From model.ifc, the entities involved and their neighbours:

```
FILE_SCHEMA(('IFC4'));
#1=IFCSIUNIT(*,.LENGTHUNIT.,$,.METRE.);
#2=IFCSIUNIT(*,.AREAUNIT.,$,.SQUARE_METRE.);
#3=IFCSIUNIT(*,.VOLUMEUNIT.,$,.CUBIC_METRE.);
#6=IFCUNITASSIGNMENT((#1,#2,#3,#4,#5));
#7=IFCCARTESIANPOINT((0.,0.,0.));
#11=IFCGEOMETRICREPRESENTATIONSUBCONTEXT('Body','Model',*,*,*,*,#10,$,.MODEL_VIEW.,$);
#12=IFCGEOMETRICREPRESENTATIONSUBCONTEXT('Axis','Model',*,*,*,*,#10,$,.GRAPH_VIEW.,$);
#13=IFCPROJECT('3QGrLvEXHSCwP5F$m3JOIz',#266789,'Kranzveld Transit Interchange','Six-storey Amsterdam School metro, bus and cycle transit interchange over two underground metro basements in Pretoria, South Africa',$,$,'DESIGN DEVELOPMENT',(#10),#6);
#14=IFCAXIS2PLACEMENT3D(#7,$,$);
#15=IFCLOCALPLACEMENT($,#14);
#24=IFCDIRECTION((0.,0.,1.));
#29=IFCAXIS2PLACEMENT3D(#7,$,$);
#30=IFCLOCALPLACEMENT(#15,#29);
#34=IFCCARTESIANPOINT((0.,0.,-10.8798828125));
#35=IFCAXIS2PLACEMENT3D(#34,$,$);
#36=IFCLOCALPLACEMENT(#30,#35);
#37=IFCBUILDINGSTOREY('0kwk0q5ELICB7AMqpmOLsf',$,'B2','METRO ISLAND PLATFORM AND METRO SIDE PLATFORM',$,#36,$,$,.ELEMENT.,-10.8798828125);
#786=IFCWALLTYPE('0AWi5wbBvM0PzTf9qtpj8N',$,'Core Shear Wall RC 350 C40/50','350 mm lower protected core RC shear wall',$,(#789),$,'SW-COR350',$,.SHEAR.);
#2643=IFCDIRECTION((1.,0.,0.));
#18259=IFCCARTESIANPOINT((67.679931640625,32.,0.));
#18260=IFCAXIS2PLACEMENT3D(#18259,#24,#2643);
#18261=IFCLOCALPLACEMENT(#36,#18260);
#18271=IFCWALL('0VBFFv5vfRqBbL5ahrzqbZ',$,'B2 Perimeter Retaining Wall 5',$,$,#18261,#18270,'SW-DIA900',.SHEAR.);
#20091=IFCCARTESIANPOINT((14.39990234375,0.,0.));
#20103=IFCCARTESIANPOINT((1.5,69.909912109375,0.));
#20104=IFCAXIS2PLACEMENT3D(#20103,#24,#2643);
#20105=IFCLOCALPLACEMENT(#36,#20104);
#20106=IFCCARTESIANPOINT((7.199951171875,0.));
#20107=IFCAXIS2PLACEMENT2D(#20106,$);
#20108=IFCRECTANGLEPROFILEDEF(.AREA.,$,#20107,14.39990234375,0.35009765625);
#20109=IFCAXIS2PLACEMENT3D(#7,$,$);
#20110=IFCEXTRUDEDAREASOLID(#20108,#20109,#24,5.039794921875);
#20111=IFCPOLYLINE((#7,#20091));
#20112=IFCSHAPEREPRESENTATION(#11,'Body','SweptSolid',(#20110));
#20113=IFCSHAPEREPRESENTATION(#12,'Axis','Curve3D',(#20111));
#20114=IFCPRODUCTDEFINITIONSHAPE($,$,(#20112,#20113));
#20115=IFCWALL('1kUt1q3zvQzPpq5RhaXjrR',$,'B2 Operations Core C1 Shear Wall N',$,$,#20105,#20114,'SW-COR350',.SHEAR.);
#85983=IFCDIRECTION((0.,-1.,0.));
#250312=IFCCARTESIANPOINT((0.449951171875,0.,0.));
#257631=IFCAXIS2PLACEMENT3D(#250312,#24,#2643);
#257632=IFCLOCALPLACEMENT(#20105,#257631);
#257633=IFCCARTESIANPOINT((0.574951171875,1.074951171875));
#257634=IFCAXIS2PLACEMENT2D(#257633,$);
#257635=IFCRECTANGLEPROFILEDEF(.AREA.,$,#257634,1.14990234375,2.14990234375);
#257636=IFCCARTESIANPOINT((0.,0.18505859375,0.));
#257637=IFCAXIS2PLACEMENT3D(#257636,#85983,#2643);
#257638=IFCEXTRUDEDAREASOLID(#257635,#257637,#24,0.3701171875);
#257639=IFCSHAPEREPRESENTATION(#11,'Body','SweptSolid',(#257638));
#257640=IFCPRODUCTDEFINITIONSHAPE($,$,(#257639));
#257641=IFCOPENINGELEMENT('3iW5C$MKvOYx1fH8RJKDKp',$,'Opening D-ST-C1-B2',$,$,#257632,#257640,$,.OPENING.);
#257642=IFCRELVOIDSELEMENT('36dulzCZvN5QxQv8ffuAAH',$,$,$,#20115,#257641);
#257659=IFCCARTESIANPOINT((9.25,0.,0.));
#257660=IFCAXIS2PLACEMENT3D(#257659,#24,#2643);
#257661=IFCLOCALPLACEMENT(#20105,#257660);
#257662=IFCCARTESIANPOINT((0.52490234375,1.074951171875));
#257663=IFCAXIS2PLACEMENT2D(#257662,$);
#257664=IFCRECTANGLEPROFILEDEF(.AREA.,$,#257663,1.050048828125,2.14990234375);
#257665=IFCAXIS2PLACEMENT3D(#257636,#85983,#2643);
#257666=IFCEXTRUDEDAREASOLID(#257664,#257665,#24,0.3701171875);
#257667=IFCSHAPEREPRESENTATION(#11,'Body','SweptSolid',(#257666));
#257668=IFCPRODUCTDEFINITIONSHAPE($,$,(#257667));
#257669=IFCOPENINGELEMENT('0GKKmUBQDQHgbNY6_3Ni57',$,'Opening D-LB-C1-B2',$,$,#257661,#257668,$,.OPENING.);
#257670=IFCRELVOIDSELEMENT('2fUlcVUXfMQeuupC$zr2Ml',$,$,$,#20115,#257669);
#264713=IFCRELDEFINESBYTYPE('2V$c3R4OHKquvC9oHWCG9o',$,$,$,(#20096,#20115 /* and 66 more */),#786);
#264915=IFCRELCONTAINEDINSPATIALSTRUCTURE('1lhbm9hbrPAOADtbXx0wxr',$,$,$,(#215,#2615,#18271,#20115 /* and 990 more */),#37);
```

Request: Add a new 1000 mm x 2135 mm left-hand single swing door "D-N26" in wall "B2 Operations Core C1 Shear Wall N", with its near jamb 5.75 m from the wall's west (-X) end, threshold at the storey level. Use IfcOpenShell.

```python
import numpy as np
import ifcopenshell
import ifcopenshell.api.feature
import ifcopenshell.api.geometry
import ifcopenshell.api.root
import ifcopenshell.api.spatial
import ifcopenshell.geom
import ifcopenshell.util.element
import ifcopenshell.util.placement
import ifcopenshell.util.representation
import ifcopenshell.util.shape
import ifcopenshell.util.unit

model = ifcopenshell.open("model.ifc")
unit_scale = ifcopenshell.util.unit.calculate_unit_scale(model)
settings = ifcopenshell.geom.settings()


def volume(element):
    """Net volume in cubic metres, openings subtracted."""
    shape = ifcopenshell.geom.create_shape(settings, element)
    return ifcopenshell.util.shape.get_volume(shape.geometry)


wall = model.by_id(20115)
storey = ifcopenshell.util.element.get_container(wall, ifc_class="IfcBuildingStorey")
context = ifcopenshell.util.representation.get_context(model, "Model", "Body", "MODEL_VIEW")
before = volume(wall)

width, height, from_end, sill = 1, 2.135, 5.75, 0.0  # metres

# The wall runs along its own X axis, and the end named is its -X end.
wall_shape = ifcopenshell.geom.create_shape(settings, wall)
x, y, z = ifcopenshell.util.shape.get_vertices(wall_shape.geometry).T
start = x.min() + from_end
face, thickness = float(y.min()), float(y.max() - y.min())
wall_matrix = ifcopenshell.util.placement.get_local_placement(wall.ObjectPlacement)
level = ifcopenshell.util.placement.get_local_placement(storey.ObjectPlacement)[2, 3]


def in_wall(x, y):
    """Placement at x, y metres in the wall's axes, at sill height."""
    matrix = wall_matrix.copy()
    matrix[:, 3] = wall_matrix @ np.array([x / unit_scale, y / unit_scale, 0.0, 1.0])
    matrix[2, 3] = level + sill / unit_scale
    return matrix


# Opening: a box that overshoots both wall faces by 50 mm.
opening = ifcopenshell.api.root.create_entity(model, ifc_class="IfcOpeningElement", predefined_type="OPENING")
box = ifcopenshell.api.geometry.add_wall_representation(
    model, context=context, length=width, height=height, thickness=thickness + 0.1
)
ifcopenshell.api.geometry.assign_representation(model, product=opening, representation=box)
ifcopenshell.api.geometry.edit_object_placement(model, product=opening, matrix=in_wall(start, face - 0.05), is_si=False)
ifcopenshell.api.feature.add_feature(model, feature=opening, element=wall)

door = ifcopenshell.api.root.create_entity(model, ifc_class="IfcDoor", name="D-N26", predefined_type="DOOR")
door.OverallWidth, door.OverallHeight = width / unit_scale, height / unit_scale
door.OperationType = "SINGLE_SWING_LEFT"
body = ifcopenshell.api.geometry.add_door_representation(
    model,
    context=context,
    overall_width=door.OverallWidth,
    overall_height=door.OverallHeight,
    operation_type="SINGLE_SWING_LEFT",
    lining_properties={"LiningDepth": thickness / unit_scale, "ThresholdDepth": thickness / unit_scale},
)
ifcopenshell.api.geometry.assign_representation(model, product=door, representation=body)
ifcopenshell.api.spatial.assign_container(model, products=[door], relating_structure=storey)
ifcopenshell.api.feature.add_filling(model, opening=opening, element=door)

# The lining spans the wall, so the door starts at the wall face.
ifcopenshell.api.geometry.edit_object_placement(model, product=door, matrix=in_wall(start, face), is_si=False)

after = volume(wall)

print(f"wall volume {before:.3f} -> {after:.3f} m3")

model.write("model-out.ifc")
```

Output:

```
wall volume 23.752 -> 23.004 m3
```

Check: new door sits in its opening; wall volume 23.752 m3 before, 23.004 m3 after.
